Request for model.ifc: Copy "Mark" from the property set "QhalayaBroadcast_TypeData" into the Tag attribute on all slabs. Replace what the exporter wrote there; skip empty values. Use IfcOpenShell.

First a look at what the model holds.

```python
import ifcopenshell
import ifcopenshell.util.element

model = ifcopenshell.open("model.ifc")
print(model.schema)
slabs = model.by_type("IfcSlab")
print(len(slabs), "slabs")
for e in slabs[:8]:
    source = ifcopenshell.util.element.get_pset(e, "QhalayaBroadcast_TypeData", "Mark")
    target = e.Tag
    print(e.id(), repr(source), repr(target), sep=" | ")
```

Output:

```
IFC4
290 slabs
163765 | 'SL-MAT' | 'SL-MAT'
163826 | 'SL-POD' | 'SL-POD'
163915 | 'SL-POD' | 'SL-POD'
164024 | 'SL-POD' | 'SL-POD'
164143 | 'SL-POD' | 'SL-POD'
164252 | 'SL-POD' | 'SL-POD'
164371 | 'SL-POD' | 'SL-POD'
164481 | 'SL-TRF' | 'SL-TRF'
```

```python
import ifcopenshell
import ifcopenshell.util.element

model = ifcopenshell.open("model.ifc")

count = 0
for e in model.by_type("IfcSlab"):
    value = ifcopenshell.util.element.get_pset(e, "QhalayaBroadcast_TypeData", "Mark")
    current = e.Tag
    if not value or not value.strip() or current == value:
        continue
    e.Tag = value
    count += 1

print(count, "slabs updated")

model.write("model_edited.ifc")
```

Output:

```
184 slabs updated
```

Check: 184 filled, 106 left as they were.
